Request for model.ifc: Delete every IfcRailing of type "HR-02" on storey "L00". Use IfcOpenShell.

First a look at what the model holds.

```python
import ifcopenshell
import ifcopenshell.util.element

model = ifcopenshell.open("model.ifc")
print(model.schema)
storey = next(s for s in model.by_type("IfcBuildingStorey") if s.Name == "L00")
railings = [e for e in ifcopenshell.util.element.get_decomposition(storey) if e.is_a("IfcRailing")]
seen = {}
for e in railings:
    element_type = ifcopenshell.util.element.get_type(e)
    name = element_type.Name if element_type not in (None, e) else None
    seen[name] = seen.get(name, 0) + 1
for name, count in sorted(seen.items(), key=str):
    print(count, "x", name)
```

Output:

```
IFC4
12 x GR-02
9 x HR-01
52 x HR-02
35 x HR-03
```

```python
import ifcopenshell
import ifcopenshell.api.root
import ifcopenshell.util.element

model = ifcopenshell.open("model.ifc")

storey = next(s for s in model.by_type("IfcBuildingStorey") if s.Name == "L00")
railings = [e for e in ifcopenshell.util.element.get_decomposition(storey) if e.is_a("IfcRailing")]
targets = [e for e in railings if (t := ifcopenshell.util.element.get_type(e)) not in (None, e) and t.Name == "HR-02"]

for e in targets:
    ifcopenshell.api.root.remove_product(model, product=e)
print(len(targets), "removed")

model.write("model_edited.ifc")
```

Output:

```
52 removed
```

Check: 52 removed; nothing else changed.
